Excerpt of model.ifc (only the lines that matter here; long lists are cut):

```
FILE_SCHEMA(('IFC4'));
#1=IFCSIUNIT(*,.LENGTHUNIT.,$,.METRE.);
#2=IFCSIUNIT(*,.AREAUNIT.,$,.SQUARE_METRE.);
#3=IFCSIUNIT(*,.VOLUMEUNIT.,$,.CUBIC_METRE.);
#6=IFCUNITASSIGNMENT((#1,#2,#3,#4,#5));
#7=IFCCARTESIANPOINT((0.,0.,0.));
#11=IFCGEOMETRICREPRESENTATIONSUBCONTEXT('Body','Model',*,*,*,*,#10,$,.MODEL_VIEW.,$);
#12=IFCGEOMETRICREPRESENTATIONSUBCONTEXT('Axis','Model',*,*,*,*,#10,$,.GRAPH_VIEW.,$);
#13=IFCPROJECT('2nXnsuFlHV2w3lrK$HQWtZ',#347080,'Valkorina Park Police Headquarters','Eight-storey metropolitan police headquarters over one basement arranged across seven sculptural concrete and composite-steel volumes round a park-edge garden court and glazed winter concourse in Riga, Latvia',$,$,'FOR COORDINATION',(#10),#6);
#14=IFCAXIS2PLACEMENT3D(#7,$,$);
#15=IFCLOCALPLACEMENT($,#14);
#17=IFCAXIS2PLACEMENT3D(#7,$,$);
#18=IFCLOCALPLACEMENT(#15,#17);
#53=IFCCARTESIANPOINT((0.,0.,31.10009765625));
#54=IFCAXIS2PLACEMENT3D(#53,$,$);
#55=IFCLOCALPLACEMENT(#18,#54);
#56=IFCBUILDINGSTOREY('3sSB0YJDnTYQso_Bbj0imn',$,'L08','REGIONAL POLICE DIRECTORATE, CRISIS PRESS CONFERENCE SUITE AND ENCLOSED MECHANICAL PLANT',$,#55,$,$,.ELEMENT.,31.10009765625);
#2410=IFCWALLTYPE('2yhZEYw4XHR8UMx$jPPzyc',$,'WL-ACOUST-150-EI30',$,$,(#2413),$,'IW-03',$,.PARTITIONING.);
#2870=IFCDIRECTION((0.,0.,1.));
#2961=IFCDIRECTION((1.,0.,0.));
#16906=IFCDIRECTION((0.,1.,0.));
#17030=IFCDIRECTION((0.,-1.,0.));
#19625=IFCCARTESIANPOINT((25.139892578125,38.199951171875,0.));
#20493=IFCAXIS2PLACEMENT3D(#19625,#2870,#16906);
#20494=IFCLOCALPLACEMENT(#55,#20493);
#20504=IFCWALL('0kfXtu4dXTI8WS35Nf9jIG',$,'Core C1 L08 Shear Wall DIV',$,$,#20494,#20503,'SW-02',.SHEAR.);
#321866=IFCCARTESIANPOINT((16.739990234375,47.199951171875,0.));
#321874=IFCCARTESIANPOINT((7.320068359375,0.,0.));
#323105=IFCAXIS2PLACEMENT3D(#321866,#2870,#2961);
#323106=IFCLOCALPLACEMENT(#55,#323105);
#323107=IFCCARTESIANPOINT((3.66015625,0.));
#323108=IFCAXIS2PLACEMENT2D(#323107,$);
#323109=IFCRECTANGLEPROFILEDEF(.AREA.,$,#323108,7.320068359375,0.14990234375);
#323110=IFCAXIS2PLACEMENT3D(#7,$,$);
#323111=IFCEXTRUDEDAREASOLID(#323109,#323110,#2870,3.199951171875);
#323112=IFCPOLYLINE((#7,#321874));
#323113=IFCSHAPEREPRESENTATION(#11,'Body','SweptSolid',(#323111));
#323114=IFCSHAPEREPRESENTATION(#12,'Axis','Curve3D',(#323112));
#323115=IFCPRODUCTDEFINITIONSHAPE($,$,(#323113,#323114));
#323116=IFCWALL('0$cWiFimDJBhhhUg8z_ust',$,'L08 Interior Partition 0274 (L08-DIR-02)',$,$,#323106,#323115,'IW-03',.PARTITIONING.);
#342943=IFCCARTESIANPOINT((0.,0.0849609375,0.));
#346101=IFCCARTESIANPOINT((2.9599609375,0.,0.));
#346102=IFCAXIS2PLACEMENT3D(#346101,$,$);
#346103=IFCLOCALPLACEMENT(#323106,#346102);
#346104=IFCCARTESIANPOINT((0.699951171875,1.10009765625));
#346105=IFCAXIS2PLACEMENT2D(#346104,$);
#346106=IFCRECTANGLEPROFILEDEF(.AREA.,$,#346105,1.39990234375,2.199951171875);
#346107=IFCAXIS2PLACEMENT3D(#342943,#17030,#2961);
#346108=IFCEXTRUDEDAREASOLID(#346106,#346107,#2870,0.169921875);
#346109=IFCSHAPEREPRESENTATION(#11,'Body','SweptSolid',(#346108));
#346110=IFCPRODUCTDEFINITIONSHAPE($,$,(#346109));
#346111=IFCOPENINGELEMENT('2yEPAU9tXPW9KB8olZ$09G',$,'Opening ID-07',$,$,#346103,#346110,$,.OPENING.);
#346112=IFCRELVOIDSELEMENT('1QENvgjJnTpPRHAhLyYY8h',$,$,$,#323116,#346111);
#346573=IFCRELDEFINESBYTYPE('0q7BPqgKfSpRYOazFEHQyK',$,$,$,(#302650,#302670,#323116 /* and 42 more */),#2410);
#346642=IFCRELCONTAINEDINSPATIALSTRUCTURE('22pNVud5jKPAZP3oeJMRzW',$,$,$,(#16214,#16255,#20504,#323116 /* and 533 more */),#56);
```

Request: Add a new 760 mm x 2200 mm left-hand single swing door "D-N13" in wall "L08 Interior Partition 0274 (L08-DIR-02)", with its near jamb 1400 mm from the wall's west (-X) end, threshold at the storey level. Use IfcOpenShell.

```python
import numpy as np
import ifcopenshell
import ifcopenshell.api.feature
import ifcopenshell.api.geometry
import ifcopenshell.api.root
import ifcopenshell.api.spatial
import ifcopenshell.geom
import ifcopenshell.util.element
import ifcopenshell.util.placement
import ifcopenshell.util.representation
import ifcopenshell.util.shape
import ifcopenshell.util.unit

model = ifcopenshell.open("model.ifc")
unit_scale = ifcopenshell.util.unit.calculate_unit_scale(model)
settings = ifcopenshell.geom.settings()


def volume(element):
    """Net volume in cubic metres, openings subtracted."""
    shape = ifcopenshell.geom.create_shape(settings, element)
    return ifcopenshell.util.shape.get_volume(shape.geometry)


wall = model.by_guid("0$cWiFimDJBhhhUg8z_ust")
storey = ifcopenshell.util.element.get_container(wall, ifc_class="IfcBuildingStorey")
context = ifcopenshell.util.representation.get_context(model, "Model", "Body", "MODEL_VIEW")
before = volume(wall)

width, height, from_end, sill = 0.76, 2.2, 1.4, 0.0  # metres

# The wall runs along its own X axis, and the end named is its -X end.
wall_shape = ifcopenshell.geom.create_shape(settings, wall)
x, y, z = ifcopenshell.util.shape.get_vertices(wall_shape.geometry).T
start = x.min() + from_end
face, thickness = float(y.min()), float(y.max() - y.min())
wall_matrix = ifcopenshell.util.placement.get_local_placement(wall.ObjectPlacement)
level = ifcopenshell.util.placement.get_local_placement(storey.ObjectPlacement)[2, 3]


def in_wall(x, y):
    """Placement at x, y metres in the wall's axes, at sill height."""
    matrix = wall_matrix.copy()
    matrix[:, 3] = wall_matrix @ np.array([x / unit_scale, y / unit_scale, 0.0, 1.0])
    matrix[2, 3] = level + sill / unit_scale
    return matrix


# Opening: a box that overshoots both wall faces by 50 mm.
opening = ifcopenshell.api.root.create_entity(model, ifc_class="IfcOpeningElement", predefined_type="OPENING")
box = ifcopenshell.api.geometry.add_wall_representation(
    model, context=context, length=width, height=height, thickness=thickness + 0.1
)
ifcopenshell.api.geometry.assign_representation(model, product=opening, representation=box)
ifcopenshell.api.geometry.edit_object_placement(model, product=opening, matrix=in_wall(start, face - 0.05), is_si=False)
ifcopenshell.api.feature.add_feature(model, feature=opening, element=wall)

door = ifcopenshell.api.root.create_entity(model, ifc_class="IfcDoor", name="D-N13", predefined_type="DOOR")
door.OverallWidth, door.OverallHeight = width / unit_scale, height / unit_scale
door.OperationType = "SINGLE_SWING_LEFT"
body = ifcopenshell.api.geometry.add_door_representation(
    model,
    context=context,
    overall_width=door.OverallWidth,
    overall_height=door.OverallHeight,
    operation_type="SINGLE_SWING_LEFT",
    lining_properties={"LiningDepth": thickness / unit_scale, "ThresholdDepth": thickness / unit_scale},
)
ifcopenshell.api.geometry.assign_representation(model, product=door, representation=body)
ifcopenshell.api.spatial.assign_container(model, products=[door], relating_structure=storey)
ifcopenshell.api.feature.add_filling(model, opening=opening, element=door)

# The lining spans the wall, so the door starts at the wall face.
ifcopenshell.api.geometry.edit_object_placement(model, product=door, matrix=in_wall(start, face), is_si=False)

after = volume(wall)

print(f"wall volume {before:.3f} -> {after:.3f} m3")

model.write("model_v2.ifc")
```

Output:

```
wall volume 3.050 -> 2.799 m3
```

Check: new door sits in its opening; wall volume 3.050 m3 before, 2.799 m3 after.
